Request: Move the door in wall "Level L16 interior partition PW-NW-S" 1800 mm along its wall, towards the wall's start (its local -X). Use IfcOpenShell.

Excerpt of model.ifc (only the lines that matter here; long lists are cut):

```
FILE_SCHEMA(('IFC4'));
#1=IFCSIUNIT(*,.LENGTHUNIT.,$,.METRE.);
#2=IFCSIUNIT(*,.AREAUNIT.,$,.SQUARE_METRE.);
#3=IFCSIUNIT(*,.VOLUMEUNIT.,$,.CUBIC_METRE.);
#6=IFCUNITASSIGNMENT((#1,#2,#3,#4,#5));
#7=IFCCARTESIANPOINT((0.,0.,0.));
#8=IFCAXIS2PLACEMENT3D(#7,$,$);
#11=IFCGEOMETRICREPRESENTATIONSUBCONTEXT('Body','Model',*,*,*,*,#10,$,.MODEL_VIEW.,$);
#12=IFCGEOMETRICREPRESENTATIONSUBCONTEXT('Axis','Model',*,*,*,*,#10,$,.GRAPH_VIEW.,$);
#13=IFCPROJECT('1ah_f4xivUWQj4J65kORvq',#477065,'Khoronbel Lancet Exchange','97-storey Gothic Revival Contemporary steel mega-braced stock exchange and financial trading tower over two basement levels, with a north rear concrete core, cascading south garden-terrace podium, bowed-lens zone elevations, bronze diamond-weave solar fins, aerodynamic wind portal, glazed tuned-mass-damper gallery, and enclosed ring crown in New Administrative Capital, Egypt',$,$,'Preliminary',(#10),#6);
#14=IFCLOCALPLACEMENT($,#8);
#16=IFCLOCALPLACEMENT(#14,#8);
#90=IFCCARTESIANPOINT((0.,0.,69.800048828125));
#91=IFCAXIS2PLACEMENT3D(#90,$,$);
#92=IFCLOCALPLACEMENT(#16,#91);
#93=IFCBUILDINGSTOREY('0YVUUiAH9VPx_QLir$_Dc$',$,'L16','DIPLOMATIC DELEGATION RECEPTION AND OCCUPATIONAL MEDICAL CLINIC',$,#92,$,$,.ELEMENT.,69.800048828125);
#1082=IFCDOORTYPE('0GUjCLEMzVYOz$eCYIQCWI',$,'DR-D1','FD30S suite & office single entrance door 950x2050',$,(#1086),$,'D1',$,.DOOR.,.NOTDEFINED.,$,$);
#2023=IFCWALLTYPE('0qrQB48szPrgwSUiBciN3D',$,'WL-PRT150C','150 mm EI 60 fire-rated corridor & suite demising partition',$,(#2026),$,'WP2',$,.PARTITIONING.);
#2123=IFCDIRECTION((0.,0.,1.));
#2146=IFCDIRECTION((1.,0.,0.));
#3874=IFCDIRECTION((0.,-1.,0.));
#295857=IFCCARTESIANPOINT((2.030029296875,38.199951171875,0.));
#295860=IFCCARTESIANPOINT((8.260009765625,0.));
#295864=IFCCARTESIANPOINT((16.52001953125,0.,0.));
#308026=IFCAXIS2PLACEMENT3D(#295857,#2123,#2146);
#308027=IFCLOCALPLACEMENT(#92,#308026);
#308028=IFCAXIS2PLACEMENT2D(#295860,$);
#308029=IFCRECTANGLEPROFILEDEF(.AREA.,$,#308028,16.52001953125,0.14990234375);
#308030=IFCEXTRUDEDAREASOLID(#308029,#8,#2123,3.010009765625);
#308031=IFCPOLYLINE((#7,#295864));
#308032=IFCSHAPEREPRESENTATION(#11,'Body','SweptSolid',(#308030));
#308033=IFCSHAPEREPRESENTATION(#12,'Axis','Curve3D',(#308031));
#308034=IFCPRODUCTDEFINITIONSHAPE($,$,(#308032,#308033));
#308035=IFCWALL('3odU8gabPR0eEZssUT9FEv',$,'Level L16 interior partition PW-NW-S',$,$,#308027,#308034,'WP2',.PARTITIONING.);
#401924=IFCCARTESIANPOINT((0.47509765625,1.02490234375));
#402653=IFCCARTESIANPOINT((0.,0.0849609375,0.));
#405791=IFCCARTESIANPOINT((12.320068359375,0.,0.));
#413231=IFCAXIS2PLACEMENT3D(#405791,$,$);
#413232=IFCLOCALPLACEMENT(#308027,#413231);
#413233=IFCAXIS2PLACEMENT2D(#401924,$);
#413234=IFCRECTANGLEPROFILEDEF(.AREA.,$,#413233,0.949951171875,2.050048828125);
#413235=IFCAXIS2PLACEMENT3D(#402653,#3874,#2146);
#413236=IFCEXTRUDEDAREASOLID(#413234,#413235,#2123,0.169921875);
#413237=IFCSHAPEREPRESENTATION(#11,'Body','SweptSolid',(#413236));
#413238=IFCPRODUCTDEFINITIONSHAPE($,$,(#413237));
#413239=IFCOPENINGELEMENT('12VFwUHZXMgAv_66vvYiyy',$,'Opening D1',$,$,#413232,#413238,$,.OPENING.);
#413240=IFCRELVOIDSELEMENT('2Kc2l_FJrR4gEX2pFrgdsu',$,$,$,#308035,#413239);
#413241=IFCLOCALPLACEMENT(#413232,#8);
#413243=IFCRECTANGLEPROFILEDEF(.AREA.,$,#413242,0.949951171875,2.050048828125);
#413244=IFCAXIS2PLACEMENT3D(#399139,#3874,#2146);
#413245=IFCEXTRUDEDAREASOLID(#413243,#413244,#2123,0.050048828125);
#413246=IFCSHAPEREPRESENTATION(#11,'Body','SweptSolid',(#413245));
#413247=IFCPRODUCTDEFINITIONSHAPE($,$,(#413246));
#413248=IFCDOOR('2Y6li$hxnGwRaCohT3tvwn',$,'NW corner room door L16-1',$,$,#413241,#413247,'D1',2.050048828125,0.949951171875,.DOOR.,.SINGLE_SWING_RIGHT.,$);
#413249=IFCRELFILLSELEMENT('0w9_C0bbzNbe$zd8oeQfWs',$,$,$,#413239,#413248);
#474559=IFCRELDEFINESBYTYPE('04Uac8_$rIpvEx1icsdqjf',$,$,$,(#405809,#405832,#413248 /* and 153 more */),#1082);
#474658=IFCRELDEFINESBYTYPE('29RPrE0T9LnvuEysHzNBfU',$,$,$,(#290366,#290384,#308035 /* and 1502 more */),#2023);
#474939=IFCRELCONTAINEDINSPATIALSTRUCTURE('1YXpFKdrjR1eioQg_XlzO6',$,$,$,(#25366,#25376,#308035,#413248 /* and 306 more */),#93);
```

```python
import ifcopenshell
import ifcopenshell.api.geometry
import ifcopenshell.util.placement
import ifcopenshell.util.unit

model = ifcopenshell.open("model.ifc")
unit_scale = ifcopenshell.util.unit.calculate_unit_scale(model)

door = model.by_id(413248)
opening = door.FillsVoids[0].RelatingOpeningElement
wall = opening.VoidsElements[0].RelatingBuildingElement

wall_matrix = ifcopenshell.util.placement.get_local_placement(wall.ObjectPlacement)
shift = wall_matrix[:3, 0] * -1.8 / unit_scale
before = ifcopenshell.util.placement.get_local_placement(door.ObjectPlacement)[:3, 3].copy()

# The door is placed relative to its opening, so it follows when the opening moves.
matrix = ifcopenshell.util.placement.get_local_placement(opening.ObjectPlacement)
matrix[:3, 3] += shift
ifcopenshell.api.geometry.edit_object_placement(
    model, product=opening, matrix=matrix, is_si=False, should_transform_children=True
)

after = ifcopenshell.util.placement.get_local_placement(door.ObjectPlacement)[:3, 3]
print("door moved by", (after - before).round(3) + 0.0)

model.write("model_updated.ifc")
```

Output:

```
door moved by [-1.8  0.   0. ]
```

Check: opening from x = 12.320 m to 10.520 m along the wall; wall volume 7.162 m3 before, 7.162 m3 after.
